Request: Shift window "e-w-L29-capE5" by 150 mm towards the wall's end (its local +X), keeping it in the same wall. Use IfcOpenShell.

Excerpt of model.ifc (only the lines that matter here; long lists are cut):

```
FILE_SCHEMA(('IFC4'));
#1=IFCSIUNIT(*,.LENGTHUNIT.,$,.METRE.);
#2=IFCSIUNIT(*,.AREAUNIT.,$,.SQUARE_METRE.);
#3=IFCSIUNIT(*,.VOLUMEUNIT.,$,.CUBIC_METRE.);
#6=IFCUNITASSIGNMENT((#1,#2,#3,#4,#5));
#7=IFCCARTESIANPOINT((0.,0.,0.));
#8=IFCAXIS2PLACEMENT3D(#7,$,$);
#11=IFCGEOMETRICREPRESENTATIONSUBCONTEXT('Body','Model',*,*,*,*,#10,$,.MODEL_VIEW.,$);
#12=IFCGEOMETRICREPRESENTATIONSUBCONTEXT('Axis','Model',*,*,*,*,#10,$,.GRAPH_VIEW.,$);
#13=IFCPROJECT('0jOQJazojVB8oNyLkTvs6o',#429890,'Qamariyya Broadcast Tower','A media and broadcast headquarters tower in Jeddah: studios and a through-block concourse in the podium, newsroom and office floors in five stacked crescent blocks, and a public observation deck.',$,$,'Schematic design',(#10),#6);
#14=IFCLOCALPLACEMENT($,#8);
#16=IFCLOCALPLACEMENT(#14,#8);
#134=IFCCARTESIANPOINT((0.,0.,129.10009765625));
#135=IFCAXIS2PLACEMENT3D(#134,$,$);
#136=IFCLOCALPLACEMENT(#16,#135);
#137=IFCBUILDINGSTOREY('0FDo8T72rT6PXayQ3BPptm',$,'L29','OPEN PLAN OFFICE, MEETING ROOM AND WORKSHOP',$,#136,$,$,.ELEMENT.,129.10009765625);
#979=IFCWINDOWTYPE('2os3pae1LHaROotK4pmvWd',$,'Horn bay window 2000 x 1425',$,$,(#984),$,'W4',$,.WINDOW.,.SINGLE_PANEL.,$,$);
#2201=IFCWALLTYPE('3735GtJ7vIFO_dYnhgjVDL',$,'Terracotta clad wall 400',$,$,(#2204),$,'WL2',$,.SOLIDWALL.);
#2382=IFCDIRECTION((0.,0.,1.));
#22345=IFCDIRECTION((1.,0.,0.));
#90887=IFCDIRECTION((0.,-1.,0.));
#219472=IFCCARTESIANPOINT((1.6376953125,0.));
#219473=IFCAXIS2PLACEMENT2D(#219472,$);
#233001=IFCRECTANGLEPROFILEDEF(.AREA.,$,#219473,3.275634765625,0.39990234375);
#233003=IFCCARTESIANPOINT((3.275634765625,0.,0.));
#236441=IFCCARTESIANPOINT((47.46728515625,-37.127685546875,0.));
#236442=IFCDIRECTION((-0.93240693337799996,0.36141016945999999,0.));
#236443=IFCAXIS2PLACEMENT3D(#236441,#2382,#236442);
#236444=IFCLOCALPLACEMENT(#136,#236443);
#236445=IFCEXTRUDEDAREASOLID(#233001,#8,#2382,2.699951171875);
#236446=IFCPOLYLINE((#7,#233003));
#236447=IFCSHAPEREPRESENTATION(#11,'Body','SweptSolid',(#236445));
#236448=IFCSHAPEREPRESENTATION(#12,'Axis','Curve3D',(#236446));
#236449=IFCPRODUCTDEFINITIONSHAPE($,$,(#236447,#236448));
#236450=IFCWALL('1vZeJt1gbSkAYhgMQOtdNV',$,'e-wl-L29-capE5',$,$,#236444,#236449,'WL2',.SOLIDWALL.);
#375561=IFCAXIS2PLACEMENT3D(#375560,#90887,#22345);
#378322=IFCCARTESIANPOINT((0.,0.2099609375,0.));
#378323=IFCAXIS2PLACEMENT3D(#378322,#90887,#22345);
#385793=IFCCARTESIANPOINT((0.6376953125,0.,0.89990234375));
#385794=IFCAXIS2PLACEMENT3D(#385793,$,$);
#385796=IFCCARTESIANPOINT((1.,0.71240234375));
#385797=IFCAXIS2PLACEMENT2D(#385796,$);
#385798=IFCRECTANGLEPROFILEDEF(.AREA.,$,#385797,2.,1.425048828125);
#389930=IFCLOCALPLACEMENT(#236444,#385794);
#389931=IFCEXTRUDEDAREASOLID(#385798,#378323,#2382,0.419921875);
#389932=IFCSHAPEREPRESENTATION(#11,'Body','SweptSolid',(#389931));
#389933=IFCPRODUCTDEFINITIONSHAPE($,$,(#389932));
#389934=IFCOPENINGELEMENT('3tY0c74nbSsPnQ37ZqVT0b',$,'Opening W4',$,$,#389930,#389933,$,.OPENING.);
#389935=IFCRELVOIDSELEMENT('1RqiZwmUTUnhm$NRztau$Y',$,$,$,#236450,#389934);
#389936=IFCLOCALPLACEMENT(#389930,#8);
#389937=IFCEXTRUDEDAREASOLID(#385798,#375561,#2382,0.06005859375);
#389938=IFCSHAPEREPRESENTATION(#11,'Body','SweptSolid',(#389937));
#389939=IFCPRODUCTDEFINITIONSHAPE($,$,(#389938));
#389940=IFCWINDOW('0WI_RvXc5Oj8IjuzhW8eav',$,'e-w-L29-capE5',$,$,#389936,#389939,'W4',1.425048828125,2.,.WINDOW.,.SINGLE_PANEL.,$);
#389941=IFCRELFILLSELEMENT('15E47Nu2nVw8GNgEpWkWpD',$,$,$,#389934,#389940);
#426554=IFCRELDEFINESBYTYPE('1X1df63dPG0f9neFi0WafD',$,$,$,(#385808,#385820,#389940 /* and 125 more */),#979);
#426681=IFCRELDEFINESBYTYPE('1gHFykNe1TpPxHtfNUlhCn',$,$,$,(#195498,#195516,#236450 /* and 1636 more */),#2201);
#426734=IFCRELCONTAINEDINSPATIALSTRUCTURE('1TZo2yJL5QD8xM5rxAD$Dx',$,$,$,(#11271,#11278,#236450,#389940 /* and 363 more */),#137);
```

```python
import ifcopenshell
import ifcopenshell.api.geometry
import ifcopenshell.util.placement
import ifcopenshell.util.unit

model = ifcopenshell.open("model.ifc")
unit_scale = ifcopenshell.util.unit.calculate_unit_scale(model)

window = model.by_guid("0WI_RvXc5Oj8IjuzhW8eav")
opening = window.FillsVoids[0].RelatingOpeningElement
wall = opening.VoidsElements[0].RelatingBuildingElement

wall_matrix = ifcopenshell.util.placement.get_local_placement(wall.ObjectPlacement)
shift = wall_matrix[:3, 0] * 0.15 / unit_scale
before = ifcopenshell.util.placement.get_local_placement(window.ObjectPlacement)[:3, 3].copy()

# The window is placed relative to its opening, so it follows when the opening moves.
matrix = ifcopenshell.util.placement.get_local_placement(opening.ObjectPlacement)
matrix[:3, 3] += shift
ifcopenshell.api.geometry.edit_object_placement(
    model, product=opening, matrix=matrix, is_si=False, should_transform_children=True
)

after = ifcopenshell.util.placement.get_local_placement(window.ObjectPlacement)[:3, 3]
print("window moved by", (after - before).round(3) + 0.0)

model.write("model-out.ifc")
```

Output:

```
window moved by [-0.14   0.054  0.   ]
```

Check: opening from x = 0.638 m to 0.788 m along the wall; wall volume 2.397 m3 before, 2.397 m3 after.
